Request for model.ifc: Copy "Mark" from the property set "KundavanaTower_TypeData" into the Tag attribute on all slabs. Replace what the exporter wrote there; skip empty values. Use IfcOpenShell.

First a look at what the model holds.

```python
import ifcopenshell
import ifcopenshell.util.element

model = ifcopenshell.open("model.ifc")
print(model.schema)
slabs = model.by_type("IfcSlab")
print(len(slabs), "slabs")
for e in slabs[:8]:
    source = ifcopenshell.util.element.get_pset(e, "KundavanaTower_TypeData", "Mark")
    target = e.Tag
    print(e.id(), repr(source), repr(target), sep=" | ")
```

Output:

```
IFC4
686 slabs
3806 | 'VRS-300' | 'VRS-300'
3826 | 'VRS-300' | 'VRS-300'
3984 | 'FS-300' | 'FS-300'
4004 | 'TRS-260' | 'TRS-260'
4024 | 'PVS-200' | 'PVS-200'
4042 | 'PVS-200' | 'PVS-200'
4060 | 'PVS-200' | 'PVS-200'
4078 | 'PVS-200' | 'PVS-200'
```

```python
import ifcopenshell
import ifcopenshell.util.element

model = ifcopenshell.open("model.ifc")

count = 0
for e in model.by_type("IfcSlab"):
    value = ifcopenshell.util.element.get_pset(e, "KundavanaTower_TypeData", "Mark")
    current = e.Tag
    if not value or not value.strip() or current == value:
        continue
    e.Tag = value
    count += 1

print(count, "slabs updated")

model.write("model-out.ifc")
```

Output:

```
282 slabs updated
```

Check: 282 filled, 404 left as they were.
